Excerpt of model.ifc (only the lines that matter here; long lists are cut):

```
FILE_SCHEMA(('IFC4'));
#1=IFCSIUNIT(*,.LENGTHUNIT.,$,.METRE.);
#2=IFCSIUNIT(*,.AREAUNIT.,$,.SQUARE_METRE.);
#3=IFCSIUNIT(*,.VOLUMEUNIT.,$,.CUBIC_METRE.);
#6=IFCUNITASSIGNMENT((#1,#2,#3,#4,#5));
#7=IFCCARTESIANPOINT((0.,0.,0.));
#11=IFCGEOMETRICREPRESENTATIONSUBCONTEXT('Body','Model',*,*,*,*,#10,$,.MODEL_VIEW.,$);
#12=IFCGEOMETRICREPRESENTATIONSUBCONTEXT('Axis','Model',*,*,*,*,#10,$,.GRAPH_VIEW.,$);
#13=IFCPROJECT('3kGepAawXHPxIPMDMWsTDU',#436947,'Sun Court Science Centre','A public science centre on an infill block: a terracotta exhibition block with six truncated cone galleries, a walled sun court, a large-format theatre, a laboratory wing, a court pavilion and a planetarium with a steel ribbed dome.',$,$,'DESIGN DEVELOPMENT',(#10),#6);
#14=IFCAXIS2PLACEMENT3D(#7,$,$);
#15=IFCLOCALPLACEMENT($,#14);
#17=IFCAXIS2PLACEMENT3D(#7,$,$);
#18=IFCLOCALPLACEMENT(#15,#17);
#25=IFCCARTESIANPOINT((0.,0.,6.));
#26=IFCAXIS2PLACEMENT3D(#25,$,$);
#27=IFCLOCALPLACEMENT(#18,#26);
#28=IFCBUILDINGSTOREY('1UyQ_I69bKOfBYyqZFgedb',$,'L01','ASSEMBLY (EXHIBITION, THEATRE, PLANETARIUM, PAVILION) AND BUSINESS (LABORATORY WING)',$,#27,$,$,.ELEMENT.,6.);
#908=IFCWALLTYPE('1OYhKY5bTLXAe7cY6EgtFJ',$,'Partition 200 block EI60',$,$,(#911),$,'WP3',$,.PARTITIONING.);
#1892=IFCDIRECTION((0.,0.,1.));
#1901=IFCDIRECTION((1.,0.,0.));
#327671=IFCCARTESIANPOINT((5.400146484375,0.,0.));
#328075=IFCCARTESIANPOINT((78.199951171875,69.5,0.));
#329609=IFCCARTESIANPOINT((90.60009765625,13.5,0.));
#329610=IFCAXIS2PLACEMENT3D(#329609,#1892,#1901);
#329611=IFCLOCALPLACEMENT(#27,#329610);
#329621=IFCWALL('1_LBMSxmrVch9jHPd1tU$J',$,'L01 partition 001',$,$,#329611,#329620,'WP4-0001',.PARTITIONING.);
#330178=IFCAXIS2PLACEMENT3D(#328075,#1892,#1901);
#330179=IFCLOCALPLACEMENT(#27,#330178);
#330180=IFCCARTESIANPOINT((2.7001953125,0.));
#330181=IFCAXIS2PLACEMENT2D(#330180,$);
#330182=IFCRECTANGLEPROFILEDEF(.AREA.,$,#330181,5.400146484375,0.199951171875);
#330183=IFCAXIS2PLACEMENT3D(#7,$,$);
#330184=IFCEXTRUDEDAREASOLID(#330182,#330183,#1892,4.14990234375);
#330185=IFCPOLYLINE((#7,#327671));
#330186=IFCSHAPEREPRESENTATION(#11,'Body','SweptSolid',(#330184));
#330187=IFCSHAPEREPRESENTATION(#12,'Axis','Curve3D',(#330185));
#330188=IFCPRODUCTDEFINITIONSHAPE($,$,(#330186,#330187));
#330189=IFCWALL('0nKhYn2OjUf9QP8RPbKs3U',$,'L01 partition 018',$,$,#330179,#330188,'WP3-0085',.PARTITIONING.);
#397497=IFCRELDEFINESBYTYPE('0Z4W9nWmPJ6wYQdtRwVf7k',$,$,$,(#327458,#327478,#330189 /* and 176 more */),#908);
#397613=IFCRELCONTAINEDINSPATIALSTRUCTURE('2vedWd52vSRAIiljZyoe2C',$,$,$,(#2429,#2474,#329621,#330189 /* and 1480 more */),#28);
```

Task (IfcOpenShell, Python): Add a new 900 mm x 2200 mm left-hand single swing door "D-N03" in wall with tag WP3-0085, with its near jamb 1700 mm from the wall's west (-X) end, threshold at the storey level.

```python
import numpy as np
import ifcopenshell
import ifcopenshell.api.feature
import ifcopenshell.api.geometry
import ifcopenshell.api.root
import ifcopenshell.api.spatial
import ifcopenshell.geom
import ifcopenshell.util.element
import ifcopenshell.util.placement
import ifcopenshell.util.representation
import ifcopenshell.util.shape
import ifcopenshell.util.unit

model = ifcopenshell.open("model.ifc")
unit_scale = ifcopenshell.util.unit.calculate_unit_scale(model)
settings = ifcopenshell.geom.settings()


def volume(element):
    """Net volume in cubic metres, openings subtracted."""
    shape = ifcopenshell.geom.create_shape(settings, element)
    return ifcopenshell.util.shape.get_volume(shape.geometry)


wall = model.by_guid("0nKhYn2OjUf9QP8RPbKs3U")
storey = ifcopenshell.util.element.get_container(wall, ifc_class="IfcBuildingStorey")
context = ifcopenshell.util.representation.get_context(model, "Model", "Body", "MODEL_VIEW")
before = volume(wall)

width, height, from_end, sill = 0.9, 2.2, 1.7, 0.0  # metres

# The wall runs along its own X axis, and the end named is its -X end.
wall_shape = ifcopenshell.geom.create_shape(settings, wall)
x, y, z = ifcopenshell.util.shape.get_vertices(wall_shape.geometry).T
start = x.min() + from_end
face, thickness = float(y.min()), float(y.max() - y.min())
wall_matrix = ifcopenshell.util.placement.get_local_placement(wall.ObjectPlacement)
level = ifcopenshell.util.placement.get_local_placement(storey.ObjectPlacement)[2, 3]


def in_wall(x, y):
    """Placement at x, y metres in the wall's axes, at sill height."""
    matrix = wall_matrix.copy()
    matrix[:, 3] = wall_matrix @ np.array([x / unit_scale, y / unit_scale, 0.0, 1.0])
    matrix[2, 3] = level + sill / unit_scale
    return matrix


# Opening: a box that overshoots both wall faces by 50 mm.
opening = ifcopenshell.api.root.create_entity(model, ifc_class="IfcOpeningElement", predefined_type="OPENING")
box = ifcopenshell.api.geometry.add_wall_representation(
    model, context=context, length=width, height=height, thickness=thickness + 0.1
)
ifcopenshell.api.geometry.assign_representation(model, product=opening, representation=box)
ifcopenshell.api.geometry.edit_object_placement(model, product=opening, matrix=in_wall(start, face - 0.05), is_si=False)
ifcopenshell.api.feature.add_feature(model, feature=opening, element=wall)

door = ifcopenshell.api.root.create_entity(model, ifc_class="IfcDoor", name="D-N03", predefined_type="DOOR")
door.OverallWidth, door.OverallHeight = width / unit_scale, height / unit_scale
door.OperationType = "SINGLE_SWING_LEFT"
body = ifcopenshell.api.geometry.add_door_representation(
    model,
    context=context,
    overall_width=door.OverallWidth,
    overall_height=door.OverallHeight,
    operation_type="SINGLE_SWING_LEFT",
    lining_properties={"LiningDepth": thickness / unit_scale, "ThresholdDepth": thickness / unit_scale},
)
ifcopenshell.api.geometry.assign_representation(model, product=door, representation=body)
ifcopenshell.api.spatial.assign_container(model, products=[door], relating_structure=storey)
ifcopenshell.api.feature.add_filling(model, opening=opening, element=door)

# The lining spans the wall, so the door starts at the wall face.
ifcopenshell.api.geometry.edit_object_placement(model, product=door, matrix=in_wall(start, face), is_si=False)

after = volume(wall)

print(f"wall volume {before:.3f} -> {after:.3f} m3")

model.write("model_rev.ifc")
```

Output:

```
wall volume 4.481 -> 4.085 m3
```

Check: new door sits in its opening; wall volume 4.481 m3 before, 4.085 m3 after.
